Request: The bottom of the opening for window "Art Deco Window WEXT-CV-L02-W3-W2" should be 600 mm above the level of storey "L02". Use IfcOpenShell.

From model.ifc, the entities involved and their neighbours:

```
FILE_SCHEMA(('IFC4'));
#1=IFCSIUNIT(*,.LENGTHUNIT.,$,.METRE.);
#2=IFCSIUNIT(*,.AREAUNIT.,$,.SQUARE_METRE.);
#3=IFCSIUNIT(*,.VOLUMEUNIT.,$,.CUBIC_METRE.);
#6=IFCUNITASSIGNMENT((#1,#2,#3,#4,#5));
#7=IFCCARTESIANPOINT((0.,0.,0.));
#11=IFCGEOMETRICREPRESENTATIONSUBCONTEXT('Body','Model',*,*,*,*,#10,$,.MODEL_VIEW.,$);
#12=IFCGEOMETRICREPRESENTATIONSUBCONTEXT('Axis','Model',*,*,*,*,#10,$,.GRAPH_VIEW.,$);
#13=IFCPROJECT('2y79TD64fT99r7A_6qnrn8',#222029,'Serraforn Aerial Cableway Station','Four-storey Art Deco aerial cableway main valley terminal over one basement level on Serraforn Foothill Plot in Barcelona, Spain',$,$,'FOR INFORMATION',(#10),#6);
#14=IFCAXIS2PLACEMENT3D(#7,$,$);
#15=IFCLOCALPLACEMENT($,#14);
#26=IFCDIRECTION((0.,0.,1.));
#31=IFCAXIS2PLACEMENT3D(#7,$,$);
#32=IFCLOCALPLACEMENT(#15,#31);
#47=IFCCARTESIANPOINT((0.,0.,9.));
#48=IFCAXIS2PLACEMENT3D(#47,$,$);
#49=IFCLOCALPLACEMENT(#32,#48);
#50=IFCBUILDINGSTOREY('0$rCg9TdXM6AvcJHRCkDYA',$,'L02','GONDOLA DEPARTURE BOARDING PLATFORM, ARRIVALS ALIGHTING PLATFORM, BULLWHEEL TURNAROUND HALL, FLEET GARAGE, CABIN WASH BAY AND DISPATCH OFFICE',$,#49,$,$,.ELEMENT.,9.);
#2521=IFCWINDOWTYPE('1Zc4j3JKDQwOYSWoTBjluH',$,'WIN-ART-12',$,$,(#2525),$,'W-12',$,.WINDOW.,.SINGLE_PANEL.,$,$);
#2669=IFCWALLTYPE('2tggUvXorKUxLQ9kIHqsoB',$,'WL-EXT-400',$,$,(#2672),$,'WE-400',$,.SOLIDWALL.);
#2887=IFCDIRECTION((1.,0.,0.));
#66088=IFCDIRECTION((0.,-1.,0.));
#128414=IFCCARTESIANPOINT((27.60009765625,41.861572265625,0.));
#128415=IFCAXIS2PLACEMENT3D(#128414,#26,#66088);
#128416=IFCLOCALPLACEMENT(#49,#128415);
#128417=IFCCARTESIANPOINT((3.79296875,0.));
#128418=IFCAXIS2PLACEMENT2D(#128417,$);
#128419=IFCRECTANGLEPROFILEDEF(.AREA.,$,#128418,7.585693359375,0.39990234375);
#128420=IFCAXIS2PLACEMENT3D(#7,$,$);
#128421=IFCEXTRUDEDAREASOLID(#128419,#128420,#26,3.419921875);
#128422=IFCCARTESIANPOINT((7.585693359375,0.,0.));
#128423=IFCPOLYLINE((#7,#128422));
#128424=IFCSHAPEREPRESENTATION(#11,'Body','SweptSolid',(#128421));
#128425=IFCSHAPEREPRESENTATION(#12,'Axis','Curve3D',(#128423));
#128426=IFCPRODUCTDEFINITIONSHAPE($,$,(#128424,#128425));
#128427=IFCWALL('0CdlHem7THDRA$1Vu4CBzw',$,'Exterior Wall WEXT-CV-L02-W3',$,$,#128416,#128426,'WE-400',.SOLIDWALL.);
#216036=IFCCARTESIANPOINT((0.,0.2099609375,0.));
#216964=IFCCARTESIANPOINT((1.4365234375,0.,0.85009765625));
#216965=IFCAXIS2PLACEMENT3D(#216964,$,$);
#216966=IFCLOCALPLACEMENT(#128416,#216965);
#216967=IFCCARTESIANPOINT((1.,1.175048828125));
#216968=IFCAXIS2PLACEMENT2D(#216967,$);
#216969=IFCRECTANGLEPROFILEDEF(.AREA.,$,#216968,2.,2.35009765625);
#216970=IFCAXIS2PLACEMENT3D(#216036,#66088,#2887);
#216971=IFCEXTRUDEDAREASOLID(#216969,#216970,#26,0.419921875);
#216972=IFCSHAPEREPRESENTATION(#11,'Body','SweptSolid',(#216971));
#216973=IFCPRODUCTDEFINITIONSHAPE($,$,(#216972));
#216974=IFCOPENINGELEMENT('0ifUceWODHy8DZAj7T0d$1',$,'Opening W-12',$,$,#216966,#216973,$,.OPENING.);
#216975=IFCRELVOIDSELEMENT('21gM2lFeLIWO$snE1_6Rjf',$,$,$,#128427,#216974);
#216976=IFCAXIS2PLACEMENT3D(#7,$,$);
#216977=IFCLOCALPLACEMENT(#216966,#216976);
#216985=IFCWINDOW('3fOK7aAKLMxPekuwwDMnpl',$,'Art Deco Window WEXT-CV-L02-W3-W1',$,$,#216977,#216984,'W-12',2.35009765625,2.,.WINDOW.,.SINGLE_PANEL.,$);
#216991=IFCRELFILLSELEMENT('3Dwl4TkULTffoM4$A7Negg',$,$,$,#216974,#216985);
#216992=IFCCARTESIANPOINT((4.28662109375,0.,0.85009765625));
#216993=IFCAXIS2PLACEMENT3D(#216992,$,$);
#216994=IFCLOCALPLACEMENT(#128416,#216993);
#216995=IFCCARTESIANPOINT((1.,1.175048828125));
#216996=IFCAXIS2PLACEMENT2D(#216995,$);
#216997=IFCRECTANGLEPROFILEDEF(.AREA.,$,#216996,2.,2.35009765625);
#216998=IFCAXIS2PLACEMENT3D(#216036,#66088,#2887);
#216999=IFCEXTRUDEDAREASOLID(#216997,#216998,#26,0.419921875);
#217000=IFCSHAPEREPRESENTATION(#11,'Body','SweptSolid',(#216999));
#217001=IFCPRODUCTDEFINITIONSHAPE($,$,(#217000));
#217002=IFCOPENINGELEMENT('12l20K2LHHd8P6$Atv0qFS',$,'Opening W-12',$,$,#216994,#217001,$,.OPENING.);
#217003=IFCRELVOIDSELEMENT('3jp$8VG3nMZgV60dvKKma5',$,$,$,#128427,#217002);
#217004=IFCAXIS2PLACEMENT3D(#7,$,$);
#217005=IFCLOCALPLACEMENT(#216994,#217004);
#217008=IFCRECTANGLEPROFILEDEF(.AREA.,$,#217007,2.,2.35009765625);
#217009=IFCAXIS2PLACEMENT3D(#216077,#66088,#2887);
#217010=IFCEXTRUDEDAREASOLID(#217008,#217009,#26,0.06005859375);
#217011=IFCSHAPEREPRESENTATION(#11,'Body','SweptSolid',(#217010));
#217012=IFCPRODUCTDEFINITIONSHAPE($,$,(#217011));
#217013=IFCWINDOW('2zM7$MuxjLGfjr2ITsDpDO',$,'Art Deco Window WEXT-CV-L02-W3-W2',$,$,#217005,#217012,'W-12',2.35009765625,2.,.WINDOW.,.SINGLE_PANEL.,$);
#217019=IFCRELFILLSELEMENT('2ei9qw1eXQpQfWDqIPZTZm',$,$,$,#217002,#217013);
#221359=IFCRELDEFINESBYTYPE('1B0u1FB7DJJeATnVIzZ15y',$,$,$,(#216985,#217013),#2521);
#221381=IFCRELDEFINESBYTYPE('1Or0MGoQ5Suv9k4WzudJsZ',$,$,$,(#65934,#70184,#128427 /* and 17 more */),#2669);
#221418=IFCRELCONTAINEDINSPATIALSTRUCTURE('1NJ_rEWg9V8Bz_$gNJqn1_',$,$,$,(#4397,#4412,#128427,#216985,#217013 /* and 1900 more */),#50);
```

```python
import numpy as np
import ifcopenshell
import ifcopenshell.api.geometry
import ifcopenshell.geom
import ifcopenshell.util.element
import ifcopenshell.util.placement
import ifcopenshell.util.shape
import ifcopenshell.util.unit

model = ifcopenshell.open("model.ifc")
unit_scale = ifcopenshell.util.unit.calculate_unit_scale(model)

window = model.by_guid("2zM7$MuxjLGfjr2ITsDpDO")
opening = window.FillsVoids[0].RelatingOpeningElement
storey = ifcopenshell.util.element.get_container(window, ifc_class="IfcBuildingStorey")
level = ifcopenshell.util.placement.get_local_placement(storey.ObjectPlacement)[2, 3]

# The opening's origin need not be at the sill, so measure its lowest point.
shape = ifcopenshell.geom.create_shape(ifcopenshell.geom.settings(), opening)
bottom = ifcopenshell.util.shape.get_shape_bottom_elevation(shape, shape.geometry) / unit_scale
dz = level + 0.6 / unit_scale - bottom

shift = np.array([0.0, 0.0, dz])
# The window is placed relative to its opening, so it follows when the opening moves.
matrix = ifcopenshell.util.placement.get_local_placement(opening.ObjectPlacement)
matrix[:3, 3] += shift
ifcopenshell.api.geometry.edit_object_placement(
    model, product=opening, matrix=matrix, is_si=False, should_transform_children=True
)

print(f"moved by {dz * unit_scale:+.3f} m")

model.write("model_v2.ifc")
```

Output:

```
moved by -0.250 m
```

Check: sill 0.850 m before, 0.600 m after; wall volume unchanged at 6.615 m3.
